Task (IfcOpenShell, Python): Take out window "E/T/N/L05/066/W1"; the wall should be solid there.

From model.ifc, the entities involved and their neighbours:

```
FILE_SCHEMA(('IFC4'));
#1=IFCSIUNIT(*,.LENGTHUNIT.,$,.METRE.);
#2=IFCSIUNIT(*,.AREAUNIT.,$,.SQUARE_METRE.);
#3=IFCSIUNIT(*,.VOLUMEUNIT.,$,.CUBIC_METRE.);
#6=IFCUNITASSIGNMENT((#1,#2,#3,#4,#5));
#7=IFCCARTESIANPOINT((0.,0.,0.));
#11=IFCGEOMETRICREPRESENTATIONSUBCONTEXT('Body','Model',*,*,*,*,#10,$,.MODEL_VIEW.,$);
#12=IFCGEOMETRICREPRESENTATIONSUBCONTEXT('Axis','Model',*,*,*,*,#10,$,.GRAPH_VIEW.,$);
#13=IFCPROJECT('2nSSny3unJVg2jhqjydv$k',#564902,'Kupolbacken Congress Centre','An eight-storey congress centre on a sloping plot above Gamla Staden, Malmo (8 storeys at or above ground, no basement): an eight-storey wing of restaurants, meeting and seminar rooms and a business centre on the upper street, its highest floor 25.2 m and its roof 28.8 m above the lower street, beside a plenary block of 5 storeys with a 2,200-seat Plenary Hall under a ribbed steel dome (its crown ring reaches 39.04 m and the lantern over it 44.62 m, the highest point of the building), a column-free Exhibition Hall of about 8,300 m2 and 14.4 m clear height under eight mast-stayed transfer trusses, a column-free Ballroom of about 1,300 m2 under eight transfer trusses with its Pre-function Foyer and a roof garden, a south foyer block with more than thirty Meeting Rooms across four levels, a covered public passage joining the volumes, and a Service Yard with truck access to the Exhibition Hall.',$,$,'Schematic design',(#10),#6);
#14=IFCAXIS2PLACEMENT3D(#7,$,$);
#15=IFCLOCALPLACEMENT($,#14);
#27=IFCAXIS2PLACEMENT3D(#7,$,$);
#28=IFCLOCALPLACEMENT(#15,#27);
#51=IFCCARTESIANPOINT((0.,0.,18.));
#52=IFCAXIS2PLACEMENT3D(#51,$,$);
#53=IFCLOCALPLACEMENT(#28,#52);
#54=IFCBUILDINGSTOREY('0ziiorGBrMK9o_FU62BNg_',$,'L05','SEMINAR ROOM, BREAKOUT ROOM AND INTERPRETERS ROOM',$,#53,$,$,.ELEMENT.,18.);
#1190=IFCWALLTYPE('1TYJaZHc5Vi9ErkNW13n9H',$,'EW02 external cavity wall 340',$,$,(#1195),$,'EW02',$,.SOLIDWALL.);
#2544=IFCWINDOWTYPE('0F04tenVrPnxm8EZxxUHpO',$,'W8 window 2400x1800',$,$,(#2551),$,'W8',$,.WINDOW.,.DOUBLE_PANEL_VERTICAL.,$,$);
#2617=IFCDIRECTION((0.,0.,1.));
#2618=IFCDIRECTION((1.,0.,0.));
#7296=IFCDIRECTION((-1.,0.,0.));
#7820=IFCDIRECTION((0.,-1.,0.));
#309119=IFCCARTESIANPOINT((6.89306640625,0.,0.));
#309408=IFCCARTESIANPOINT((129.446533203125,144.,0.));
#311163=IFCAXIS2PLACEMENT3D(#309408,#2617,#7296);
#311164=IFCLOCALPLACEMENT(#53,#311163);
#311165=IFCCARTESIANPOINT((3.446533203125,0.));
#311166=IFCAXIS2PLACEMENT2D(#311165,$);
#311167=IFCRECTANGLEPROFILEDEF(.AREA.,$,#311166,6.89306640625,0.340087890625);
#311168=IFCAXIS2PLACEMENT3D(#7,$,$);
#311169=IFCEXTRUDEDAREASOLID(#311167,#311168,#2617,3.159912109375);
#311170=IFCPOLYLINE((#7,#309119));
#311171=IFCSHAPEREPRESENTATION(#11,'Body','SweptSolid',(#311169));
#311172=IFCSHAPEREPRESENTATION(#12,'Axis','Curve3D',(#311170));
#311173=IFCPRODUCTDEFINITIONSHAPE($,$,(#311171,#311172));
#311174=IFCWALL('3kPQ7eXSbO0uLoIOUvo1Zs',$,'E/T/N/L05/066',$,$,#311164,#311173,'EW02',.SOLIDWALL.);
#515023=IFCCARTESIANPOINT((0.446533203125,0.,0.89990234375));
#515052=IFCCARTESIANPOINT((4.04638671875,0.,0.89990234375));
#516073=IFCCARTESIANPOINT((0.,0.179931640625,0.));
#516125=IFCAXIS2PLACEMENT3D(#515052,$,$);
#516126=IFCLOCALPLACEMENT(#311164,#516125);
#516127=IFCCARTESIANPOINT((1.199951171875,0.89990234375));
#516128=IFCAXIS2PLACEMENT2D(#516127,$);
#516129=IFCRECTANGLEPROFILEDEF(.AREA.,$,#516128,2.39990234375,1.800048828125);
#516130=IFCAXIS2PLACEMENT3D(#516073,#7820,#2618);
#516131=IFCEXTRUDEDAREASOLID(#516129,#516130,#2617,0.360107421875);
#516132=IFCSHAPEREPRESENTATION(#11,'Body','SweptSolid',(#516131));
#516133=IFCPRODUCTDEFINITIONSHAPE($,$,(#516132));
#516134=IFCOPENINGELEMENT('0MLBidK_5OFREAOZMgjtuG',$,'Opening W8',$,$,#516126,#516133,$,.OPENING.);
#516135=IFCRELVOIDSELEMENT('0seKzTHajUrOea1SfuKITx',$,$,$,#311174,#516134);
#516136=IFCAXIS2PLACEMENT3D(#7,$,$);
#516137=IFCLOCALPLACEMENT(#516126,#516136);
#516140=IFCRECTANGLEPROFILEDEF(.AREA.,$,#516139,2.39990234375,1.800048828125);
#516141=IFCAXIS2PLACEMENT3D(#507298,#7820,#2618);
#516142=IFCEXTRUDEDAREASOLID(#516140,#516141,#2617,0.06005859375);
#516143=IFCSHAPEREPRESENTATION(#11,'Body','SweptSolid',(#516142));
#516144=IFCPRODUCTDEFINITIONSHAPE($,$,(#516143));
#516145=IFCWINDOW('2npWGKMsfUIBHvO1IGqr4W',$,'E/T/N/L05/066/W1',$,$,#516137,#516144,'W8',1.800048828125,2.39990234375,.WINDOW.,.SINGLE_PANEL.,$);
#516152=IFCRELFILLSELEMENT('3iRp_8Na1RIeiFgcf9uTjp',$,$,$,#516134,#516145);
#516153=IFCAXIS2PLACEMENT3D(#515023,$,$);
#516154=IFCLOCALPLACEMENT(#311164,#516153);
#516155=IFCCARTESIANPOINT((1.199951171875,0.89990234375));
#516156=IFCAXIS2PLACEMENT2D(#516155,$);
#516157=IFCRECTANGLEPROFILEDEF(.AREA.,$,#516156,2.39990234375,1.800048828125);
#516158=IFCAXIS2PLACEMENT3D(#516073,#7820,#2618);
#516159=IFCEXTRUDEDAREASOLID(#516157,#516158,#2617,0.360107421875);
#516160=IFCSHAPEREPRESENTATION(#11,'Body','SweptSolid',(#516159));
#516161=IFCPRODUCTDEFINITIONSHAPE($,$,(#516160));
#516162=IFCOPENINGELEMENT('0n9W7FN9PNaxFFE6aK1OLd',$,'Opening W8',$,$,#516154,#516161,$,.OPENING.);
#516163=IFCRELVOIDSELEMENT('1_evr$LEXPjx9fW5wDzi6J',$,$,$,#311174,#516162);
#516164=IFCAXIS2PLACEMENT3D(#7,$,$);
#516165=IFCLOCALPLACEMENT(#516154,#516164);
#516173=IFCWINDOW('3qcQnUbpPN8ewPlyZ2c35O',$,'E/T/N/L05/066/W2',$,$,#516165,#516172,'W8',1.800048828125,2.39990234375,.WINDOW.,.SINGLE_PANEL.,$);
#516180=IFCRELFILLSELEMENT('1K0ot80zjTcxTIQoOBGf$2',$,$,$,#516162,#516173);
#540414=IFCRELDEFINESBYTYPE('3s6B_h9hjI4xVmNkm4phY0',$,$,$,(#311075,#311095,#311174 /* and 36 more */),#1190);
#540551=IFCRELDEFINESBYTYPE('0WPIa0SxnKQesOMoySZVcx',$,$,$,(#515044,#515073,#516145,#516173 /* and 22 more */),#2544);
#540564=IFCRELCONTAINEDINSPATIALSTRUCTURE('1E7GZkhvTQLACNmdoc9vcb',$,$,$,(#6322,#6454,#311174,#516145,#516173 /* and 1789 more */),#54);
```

```python
import ifcopenshell
import ifcopenshell.api.feature
import ifcopenshell.api.root
import ifcopenshell.geom
import ifcopenshell.util.shape

model = ifcopenshell.open("model.ifc")
settings = ifcopenshell.geom.settings()


def volume(element):
    """Net volume in cubic metres, openings subtracted."""
    shape = ifcopenshell.geom.create_shape(settings, element)
    return ifcopenshell.util.shape.get_volume(shape.geometry)


window = model.by_guid("2npWGKMsfUIBHvO1IGqr4W")
opening = window.FillsVoids[0].RelatingOpeningElement
wall = opening.VoidsElements[0].RelatingBuildingElement
before = volume(wall)

ifcopenshell.api.root.remove_product(model, product=window)
ifcopenshell.api.feature.remove_feature(model, feature=opening)

after = volume(wall)

print(f"wall volume {before:.3f} -> {after:.3f} m3")

model.write("model-out.ifc")
```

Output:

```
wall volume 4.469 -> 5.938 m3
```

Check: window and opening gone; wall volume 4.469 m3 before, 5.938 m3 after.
